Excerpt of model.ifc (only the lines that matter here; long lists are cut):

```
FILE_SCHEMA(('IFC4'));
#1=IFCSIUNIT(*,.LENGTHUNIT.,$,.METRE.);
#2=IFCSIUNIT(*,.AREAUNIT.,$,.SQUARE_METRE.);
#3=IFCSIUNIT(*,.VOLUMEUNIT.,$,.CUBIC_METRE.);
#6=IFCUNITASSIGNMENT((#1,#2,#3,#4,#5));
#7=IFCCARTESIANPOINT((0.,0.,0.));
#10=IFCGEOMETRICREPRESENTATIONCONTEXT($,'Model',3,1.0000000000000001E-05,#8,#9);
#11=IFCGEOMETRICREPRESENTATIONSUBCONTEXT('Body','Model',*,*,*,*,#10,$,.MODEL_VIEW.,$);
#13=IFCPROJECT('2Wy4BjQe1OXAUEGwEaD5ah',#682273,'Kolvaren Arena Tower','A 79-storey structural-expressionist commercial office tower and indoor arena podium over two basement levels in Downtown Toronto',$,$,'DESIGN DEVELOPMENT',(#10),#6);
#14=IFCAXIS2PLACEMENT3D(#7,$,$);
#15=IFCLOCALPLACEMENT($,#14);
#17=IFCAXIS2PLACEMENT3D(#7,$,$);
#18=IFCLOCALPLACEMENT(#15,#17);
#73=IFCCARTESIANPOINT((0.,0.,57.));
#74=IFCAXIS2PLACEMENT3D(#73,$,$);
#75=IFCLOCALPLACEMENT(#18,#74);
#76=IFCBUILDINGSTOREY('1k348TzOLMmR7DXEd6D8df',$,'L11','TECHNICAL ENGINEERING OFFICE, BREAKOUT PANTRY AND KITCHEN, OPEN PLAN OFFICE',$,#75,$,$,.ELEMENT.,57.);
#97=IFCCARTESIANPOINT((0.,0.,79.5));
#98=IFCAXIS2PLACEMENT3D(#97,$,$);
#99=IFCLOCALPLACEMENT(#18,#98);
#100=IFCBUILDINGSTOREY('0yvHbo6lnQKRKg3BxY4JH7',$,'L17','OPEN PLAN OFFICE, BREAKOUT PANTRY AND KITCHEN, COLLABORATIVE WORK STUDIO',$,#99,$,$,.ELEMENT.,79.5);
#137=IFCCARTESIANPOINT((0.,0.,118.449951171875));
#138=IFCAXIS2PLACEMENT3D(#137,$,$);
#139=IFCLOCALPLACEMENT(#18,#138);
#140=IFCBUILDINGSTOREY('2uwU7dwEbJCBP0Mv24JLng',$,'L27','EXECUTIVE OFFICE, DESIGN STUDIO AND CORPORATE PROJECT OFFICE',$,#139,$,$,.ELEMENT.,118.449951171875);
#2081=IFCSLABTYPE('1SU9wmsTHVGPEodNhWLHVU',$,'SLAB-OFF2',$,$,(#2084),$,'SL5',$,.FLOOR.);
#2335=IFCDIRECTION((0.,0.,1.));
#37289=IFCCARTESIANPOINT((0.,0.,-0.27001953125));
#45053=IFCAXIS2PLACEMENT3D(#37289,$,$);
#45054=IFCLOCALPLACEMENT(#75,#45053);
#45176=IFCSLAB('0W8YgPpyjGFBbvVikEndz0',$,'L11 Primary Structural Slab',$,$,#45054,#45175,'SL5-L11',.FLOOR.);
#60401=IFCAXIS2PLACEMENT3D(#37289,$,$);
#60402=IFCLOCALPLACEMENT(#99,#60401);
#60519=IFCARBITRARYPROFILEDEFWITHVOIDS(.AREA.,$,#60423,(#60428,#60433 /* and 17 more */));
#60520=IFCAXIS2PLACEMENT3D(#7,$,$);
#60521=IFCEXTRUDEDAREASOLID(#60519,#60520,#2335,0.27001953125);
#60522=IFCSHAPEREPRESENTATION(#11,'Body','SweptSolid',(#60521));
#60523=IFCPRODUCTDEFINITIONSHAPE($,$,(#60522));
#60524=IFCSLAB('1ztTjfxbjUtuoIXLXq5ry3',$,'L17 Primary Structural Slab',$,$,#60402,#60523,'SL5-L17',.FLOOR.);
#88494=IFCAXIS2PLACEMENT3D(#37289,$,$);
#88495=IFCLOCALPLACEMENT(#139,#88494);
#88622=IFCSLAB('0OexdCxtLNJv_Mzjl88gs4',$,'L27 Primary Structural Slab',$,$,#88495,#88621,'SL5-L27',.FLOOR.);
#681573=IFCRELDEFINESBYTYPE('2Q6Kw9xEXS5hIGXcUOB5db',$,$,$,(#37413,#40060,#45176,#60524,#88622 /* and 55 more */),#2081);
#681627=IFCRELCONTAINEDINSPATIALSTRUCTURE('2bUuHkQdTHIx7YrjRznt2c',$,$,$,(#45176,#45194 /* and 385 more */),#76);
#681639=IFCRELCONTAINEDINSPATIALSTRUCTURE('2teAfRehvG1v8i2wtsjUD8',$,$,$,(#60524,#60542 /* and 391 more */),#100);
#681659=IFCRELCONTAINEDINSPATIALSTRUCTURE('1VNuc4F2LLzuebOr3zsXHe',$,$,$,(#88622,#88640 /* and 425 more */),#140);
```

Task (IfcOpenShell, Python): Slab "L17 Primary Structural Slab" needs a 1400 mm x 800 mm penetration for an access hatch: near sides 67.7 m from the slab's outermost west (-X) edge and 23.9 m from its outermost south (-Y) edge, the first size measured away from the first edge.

```python
import numpy as np
import ifcopenshell
import ifcopenshell.api.feature
import ifcopenshell.api.geometry
import ifcopenshell.api.root
import ifcopenshell.geom
import ifcopenshell.util.placement
import ifcopenshell.util.representation
import ifcopenshell.util.shape
import ifcopenshell.util.unit

model = ifcopenshell.open("model.ifc")
unit_scale = ifcopenshell.util.unit.calculate_unit_scale(model)
settings = ifcopenshell.geom.settings()


def volume(element):
    """Net volume in cubic metres, openings subtracted."""
    shape = ifcopenshell.geom.create_shape(settings, element)
    return ifcopenshell.util.shape.get_volume(shape.geometry)


slab = model.by_guid("1ztTjfxbjUtuoIXLXq5ry3")
before = volume(slab)

# Extent in the slab's own axes, in metres. The edges named are its -X and -Y sides.
slab_shape = ifcopenshell.geom.create_shape(settings, slab)
vertices = ifcopenshell.util.shape.get_vertices(slab_shape.geometry)
x_min, y_min, bottom = vertices.min(axis=0)
top = vertices[:, 2].max()

opening = ifcopenshell.api.root.create_entity(model, ifc_class="IfcOpeningElement", name="Access hatch opening", predefined_type="OPENING")
context = ifcopenshell.util.representation.get_context(model, "Model", "Body", "MODEL_VIEW")
width, depth = 1.4, 0.8
outline = [(0.0, 0.0), (width, 0.0), (width, depth), (0.0, depth), (0.0, 0.0)]
# Overshoot both faces by 50 mm so the cut is clean.
shape = ifcopenshell.api.geometry.add_slab_representation(
    model, context=context, depth=top - bottom + 0.1, polyline=outline
)
ifcopenshell.api.geometry.assign_representation(model, product=opening, representation=shape)

matrix = ifcopenshell.util.placement.get_local_placement(slab.ObjectPlacement)
matrix[:, 3] = matrix @ np.append(np.array([x_min + 67.7, y_min + 23.9, bottom - 0.05]) / unit_scale, 1.0)
ifcopenshell.api.geometry.edit_object_placement(model, product=opening, matrix=matrix, is_si=False)
ifcopenshell.api.feature.add_feature(model, feature=opening, element=slab)

after = volume(slab)

print(f"slab volume {before:.3f} -> {after:.3f} m3")

model.write("model_v2.ifc")
```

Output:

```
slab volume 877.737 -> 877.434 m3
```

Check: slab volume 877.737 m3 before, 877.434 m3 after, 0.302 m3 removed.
